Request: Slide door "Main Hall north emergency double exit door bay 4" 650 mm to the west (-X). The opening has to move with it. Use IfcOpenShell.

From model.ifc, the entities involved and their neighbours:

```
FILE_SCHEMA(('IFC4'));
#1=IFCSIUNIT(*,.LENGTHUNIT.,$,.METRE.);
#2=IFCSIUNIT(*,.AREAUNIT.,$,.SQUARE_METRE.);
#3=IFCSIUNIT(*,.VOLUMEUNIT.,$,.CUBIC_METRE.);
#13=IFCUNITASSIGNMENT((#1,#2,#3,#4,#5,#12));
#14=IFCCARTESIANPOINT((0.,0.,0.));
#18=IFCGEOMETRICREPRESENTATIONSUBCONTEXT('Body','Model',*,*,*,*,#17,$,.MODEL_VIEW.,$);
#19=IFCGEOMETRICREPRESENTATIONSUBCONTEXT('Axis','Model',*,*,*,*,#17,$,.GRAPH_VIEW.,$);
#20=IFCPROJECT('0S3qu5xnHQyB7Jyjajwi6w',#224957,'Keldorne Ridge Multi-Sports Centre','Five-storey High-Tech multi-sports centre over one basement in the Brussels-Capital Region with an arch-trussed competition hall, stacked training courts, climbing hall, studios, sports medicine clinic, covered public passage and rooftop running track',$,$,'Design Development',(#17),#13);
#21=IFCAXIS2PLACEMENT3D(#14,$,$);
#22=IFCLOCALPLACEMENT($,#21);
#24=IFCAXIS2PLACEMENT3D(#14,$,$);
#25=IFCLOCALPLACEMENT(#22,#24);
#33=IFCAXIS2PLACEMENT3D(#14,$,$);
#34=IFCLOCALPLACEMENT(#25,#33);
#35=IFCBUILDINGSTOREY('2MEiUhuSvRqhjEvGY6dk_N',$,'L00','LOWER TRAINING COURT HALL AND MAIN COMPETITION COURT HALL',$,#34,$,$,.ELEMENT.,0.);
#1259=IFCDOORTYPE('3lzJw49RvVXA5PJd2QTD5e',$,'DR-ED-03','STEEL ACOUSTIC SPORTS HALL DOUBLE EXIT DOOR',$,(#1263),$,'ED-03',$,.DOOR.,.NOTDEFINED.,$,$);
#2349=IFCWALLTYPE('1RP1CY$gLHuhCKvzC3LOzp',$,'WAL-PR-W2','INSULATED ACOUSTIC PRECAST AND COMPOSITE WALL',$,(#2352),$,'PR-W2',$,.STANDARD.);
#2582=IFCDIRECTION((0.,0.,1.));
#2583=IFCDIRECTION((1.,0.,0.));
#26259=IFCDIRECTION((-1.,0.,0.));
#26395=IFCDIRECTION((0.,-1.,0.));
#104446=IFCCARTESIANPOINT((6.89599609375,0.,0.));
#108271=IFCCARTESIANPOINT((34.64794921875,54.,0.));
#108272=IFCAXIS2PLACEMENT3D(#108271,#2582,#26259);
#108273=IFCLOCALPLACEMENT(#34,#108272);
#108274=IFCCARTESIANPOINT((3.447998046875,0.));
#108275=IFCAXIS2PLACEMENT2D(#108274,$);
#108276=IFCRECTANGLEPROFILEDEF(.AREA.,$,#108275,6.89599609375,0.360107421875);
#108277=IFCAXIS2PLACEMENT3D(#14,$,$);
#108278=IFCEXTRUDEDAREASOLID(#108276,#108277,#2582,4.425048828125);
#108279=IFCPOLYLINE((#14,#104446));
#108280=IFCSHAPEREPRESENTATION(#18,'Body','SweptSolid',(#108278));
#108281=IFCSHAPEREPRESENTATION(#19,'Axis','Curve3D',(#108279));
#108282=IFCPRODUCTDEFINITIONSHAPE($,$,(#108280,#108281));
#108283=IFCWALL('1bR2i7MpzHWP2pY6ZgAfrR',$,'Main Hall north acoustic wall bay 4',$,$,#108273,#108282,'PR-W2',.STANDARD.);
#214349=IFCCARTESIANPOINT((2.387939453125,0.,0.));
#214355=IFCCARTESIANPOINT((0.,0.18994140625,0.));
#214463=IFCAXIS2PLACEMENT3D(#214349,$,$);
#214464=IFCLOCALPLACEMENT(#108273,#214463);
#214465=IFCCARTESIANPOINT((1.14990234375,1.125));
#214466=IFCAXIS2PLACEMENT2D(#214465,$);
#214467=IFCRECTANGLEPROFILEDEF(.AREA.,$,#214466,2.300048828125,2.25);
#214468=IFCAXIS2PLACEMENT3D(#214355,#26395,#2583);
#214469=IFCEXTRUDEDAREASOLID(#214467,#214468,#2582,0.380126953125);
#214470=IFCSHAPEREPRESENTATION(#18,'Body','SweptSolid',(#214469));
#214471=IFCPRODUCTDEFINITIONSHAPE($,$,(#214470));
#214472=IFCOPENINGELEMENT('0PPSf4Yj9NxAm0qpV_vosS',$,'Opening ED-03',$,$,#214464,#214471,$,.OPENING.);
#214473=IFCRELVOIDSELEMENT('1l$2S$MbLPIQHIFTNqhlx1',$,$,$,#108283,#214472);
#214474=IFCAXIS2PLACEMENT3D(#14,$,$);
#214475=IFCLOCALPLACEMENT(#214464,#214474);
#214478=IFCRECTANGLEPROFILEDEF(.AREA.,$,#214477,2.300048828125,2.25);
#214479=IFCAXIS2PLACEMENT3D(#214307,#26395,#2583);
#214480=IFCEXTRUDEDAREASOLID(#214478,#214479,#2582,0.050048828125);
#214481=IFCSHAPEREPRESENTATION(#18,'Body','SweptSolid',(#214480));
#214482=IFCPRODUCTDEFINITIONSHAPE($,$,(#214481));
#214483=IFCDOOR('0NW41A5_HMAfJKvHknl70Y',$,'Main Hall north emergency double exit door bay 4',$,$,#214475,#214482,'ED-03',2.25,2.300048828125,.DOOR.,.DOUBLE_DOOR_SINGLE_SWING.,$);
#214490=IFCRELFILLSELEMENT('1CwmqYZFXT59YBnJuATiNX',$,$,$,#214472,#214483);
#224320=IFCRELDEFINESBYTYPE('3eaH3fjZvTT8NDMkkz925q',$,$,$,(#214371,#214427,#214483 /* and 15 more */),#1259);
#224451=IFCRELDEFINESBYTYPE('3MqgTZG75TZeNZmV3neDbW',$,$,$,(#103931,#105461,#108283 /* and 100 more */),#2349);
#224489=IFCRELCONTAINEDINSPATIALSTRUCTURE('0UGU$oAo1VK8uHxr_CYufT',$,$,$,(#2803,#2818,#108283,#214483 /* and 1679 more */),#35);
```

```python
import ifcopenshell
import ifcopenshell.api.geometry
import ifcopenshell.util.placement

model = ifcopenshell.open("model.ifc")

door = model.by_guid("0NW41A5_HMAfJKvHknl70Y")
opening = door.FillsVoids[0].RelatingOpeningElement
wall = opening.VoidsElements[0].RelatingBuildingElement

wall_matrix = ifcopenshell.util.placement.get_local_placement(wall.ObjectPlacement)
shift = wall_matrix[:3, 0] * 0.65
before = ifcopenshell.util.placement.get_local_placement(door.ObjectPlacement)[:3, 3].copy()

# The door is placed relative to its opening, so it follows when the opening moves.
matrix = ifcopenshell.util.placement.get_local_placement(opening.ObjectPlacement)
matrix[:3, 3] += shift
ifcopenshell.api.geometry.edit_object_placement(
    model, product=opening, matrix=matrix, is_si=False, should_transform_children=True
)

after = ifcopenshell.util.placement.get_local_placement(door.ObjectPlacement)[:3, 3]
print("door moved by", (after - before).round(3) + 0.0)

model.write("model_v2.ifc")
```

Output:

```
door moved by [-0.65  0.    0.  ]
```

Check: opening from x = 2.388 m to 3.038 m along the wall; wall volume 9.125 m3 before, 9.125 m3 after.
